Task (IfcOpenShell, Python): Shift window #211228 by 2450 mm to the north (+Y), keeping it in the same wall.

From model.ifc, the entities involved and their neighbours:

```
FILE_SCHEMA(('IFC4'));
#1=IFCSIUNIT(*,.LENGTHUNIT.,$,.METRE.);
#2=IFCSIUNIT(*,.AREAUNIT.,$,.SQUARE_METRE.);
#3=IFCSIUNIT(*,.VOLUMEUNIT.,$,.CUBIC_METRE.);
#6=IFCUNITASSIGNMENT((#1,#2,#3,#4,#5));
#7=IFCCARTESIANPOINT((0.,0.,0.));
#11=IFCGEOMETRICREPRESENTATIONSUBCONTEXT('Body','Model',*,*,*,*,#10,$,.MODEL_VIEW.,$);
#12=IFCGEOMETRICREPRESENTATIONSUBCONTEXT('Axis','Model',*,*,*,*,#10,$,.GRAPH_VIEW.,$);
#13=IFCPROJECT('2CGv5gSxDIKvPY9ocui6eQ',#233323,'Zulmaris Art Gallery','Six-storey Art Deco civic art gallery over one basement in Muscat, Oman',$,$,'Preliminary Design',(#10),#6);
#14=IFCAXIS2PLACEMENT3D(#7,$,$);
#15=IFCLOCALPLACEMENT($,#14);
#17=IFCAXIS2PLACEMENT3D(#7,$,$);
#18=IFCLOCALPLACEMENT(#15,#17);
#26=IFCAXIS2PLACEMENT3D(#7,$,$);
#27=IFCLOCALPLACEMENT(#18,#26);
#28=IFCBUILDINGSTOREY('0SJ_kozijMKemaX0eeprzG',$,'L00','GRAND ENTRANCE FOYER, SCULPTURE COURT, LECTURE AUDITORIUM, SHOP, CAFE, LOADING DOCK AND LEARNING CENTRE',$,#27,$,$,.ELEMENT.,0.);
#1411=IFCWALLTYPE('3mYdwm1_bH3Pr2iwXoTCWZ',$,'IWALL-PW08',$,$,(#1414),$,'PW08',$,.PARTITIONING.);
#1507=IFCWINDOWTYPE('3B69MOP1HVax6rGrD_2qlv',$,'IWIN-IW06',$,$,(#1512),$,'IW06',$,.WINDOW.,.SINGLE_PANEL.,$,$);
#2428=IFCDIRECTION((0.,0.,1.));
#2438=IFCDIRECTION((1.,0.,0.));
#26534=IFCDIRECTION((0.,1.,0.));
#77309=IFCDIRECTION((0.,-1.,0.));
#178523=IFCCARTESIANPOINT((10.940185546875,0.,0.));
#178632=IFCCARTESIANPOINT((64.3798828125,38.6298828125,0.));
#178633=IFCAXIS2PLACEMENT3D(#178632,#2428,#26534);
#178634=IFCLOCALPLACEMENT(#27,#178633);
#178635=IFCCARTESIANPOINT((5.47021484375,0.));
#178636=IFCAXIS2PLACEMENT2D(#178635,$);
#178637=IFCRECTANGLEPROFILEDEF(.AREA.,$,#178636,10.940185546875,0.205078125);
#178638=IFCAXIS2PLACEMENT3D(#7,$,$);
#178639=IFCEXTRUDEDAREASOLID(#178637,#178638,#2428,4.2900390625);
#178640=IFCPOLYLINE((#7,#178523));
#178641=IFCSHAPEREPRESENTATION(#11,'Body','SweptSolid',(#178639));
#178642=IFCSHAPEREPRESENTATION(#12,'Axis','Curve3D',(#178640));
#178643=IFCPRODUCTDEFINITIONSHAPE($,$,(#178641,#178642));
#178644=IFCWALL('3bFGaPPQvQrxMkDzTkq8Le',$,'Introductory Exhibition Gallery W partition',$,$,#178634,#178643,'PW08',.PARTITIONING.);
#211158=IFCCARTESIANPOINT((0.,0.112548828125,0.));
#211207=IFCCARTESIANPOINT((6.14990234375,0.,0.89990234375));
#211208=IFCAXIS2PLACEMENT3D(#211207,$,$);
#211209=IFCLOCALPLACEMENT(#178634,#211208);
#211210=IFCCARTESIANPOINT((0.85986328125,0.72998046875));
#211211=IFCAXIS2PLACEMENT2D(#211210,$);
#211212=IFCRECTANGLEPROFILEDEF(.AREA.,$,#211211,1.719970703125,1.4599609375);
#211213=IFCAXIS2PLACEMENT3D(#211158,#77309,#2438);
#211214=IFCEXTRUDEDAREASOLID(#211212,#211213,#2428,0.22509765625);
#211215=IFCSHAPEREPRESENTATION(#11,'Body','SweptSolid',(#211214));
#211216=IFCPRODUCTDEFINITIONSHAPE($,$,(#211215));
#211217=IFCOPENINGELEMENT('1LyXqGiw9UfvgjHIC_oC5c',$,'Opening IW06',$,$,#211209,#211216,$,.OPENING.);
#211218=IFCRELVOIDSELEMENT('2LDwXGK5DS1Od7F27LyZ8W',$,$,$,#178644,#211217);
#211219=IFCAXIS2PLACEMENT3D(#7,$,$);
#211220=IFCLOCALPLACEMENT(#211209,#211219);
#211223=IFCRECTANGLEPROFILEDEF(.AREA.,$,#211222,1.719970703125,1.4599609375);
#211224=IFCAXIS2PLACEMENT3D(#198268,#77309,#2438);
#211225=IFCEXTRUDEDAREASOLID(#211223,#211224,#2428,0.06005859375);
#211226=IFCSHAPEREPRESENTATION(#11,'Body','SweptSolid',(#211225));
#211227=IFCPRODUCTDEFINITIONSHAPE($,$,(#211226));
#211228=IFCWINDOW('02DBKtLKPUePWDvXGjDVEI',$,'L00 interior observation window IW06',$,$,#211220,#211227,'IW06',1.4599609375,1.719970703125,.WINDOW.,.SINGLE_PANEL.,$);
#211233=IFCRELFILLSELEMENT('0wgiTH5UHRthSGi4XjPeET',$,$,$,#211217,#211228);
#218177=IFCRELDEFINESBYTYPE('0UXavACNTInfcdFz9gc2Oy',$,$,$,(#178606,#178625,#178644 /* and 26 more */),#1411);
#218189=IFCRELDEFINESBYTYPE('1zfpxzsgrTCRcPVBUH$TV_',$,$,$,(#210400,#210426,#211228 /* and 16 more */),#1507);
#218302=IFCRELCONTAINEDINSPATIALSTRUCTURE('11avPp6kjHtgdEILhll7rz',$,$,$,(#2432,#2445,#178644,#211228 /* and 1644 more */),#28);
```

```python
import ifcopenshell
import ifcopenshell.api.geometry
import ifcopenshell.util.placement
import ifcopenshell.util.unit

model = ifcopenshell.open("model.ifc")
unit_scale = ifcopenshell.util.unit.calculate_unit_scale(model)

window = model.by_guid("02DBKtLKPUePWDvXGjDVEI")
opening = window.FillsVoids[0].RelatingOpeningElement
wall = opening.VoidsElements[0].RelatingBuildingElement

wall_matrix = ifcopenshell.util.placement.get_local_placement(wall.ObjectPlacement)
shift = wall_matrix[:3, 0] * 2.45 / unit_scale
before = ifcopenshell.util.placement.get_local_placement(window.ObjectPlacement)[:3, 3].copy()

# The window is placed relative to its opening, so it follows when the opening moves.
matrix = ifcopenshell.util.placement.get_local_placement(opening.ObjectPlacement)
matrix[:3, 3] += shift
ifcopenshell.api.geometry.edit_object_placement(
    model, product=opening, matrix=matrix, is_si=False, should_transform_children=True
)

after = ifcopenshell.util.placement.get_local_placement(window.ObjectPlacement)[:3, 3]
print("window moved by", (after - before).round(3) + 0.0)

model.write("model_updated.ifc")
```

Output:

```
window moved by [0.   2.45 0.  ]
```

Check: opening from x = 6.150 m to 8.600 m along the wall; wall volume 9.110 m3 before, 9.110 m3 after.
